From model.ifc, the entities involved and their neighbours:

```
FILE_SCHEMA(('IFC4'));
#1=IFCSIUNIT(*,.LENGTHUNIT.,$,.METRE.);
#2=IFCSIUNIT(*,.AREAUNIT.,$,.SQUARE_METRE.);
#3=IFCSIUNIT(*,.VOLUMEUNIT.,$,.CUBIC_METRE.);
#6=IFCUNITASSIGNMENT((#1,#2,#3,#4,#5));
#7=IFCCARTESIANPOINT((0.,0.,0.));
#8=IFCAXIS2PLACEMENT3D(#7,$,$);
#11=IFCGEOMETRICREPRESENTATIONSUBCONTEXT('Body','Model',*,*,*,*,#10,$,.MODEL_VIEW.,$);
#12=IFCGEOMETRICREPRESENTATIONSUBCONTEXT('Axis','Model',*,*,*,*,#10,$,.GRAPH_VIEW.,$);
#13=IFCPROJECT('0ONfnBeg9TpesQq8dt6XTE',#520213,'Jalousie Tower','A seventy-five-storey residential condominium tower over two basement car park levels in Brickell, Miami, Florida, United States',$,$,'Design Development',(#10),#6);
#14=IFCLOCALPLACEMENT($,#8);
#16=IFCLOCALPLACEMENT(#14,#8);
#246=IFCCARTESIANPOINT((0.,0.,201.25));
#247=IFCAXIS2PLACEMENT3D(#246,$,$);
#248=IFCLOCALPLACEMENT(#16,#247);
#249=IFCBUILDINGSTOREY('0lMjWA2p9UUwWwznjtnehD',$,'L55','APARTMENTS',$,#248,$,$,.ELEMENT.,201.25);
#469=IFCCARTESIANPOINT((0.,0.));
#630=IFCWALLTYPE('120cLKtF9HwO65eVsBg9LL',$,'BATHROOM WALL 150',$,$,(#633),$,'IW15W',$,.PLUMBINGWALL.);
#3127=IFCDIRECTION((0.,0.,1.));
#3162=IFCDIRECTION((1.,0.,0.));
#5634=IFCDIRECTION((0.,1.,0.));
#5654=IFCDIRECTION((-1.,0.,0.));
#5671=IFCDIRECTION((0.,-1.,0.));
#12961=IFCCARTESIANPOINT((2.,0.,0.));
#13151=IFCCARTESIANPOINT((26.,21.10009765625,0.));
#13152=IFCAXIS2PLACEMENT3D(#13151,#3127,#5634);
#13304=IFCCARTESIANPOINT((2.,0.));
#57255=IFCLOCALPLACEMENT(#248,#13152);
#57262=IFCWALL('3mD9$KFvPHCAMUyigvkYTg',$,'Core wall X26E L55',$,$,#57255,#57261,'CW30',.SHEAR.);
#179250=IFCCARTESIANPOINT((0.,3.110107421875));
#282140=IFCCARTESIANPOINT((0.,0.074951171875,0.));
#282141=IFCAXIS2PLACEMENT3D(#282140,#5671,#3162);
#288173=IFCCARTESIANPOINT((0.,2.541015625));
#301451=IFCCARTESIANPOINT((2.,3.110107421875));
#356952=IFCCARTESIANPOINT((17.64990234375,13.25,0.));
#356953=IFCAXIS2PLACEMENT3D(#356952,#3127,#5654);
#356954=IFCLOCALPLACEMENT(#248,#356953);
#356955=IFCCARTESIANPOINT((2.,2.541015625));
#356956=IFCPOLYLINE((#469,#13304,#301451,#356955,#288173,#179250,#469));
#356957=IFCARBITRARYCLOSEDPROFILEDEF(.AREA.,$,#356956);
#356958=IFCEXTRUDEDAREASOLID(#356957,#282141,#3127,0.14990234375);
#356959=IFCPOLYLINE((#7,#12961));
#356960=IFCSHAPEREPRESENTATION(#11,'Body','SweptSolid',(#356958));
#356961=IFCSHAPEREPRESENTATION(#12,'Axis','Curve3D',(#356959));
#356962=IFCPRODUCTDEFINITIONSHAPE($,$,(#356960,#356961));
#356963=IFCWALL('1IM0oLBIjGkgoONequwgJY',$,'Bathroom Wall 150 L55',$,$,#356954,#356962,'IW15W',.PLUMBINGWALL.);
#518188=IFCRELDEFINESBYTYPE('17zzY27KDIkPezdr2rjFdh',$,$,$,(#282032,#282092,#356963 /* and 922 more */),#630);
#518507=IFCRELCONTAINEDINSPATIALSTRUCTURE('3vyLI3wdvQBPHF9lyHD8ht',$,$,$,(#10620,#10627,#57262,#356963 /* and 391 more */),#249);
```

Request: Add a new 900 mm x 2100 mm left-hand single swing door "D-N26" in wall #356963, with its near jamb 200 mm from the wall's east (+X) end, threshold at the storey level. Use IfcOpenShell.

```python
import numpy as np
import ifcopenshell
import ifcopenshell.api.feature
import ifcopenshell.api.geometry
import ifcopenshell.api.root
import ifcopenshell.api.spatial
import ifcopenshell.geom
import ifcopenshell.util.element
import ifcopenshell.util.placement
import ifcopenshell.util.representation
import ifcopenshell.util.shape
import ifcopenshell.util.unit

model = ifcopenshell.open("model.ifc")
unit_scale = ifcopenshell.util.unit.calculate_unit_scale(model)
settings = ifcopenshell.geom.settings()


def volume(element):
    """Net volume in cubic metres, openings subtracted."""
    shape = ifcopenshell.geom.create_shape(settings, element)
    return ifcopenshell.util.shape.get_volume(shape.geometry)


wall = model.by_guid("1IM0oLBIjGkgoONequwgJY")
storey = ifcopenshell.util.element.get_container(wall, ifc_class="IfcBuildingStorey")
context = ifcopenshell.util.representation.get_context(model, "Model", "Body", "MODEL_VIEW")
before = volume(wall)

width, height, from_end, sill = 0.9, 2.1, 0.2, 0.0  # metres

# The wall runs along its own X axis, and the end named is its -X end.
wall_shape = ifcopenshell.geom.create_shape(settings, wall)
x, y, z = ifcopenshell.util.shape.get_vertices(wall_shape.geometry).T
start = x.min() + from_end
face, thickness = float(y.min()), float(y.max() - y.min())
wall_matrix = ifcopenshell.util.placement.get_local_placement(wall.ObjectPlacement)
level = ifcopenshell.util.placement.get_local_placement(storey.ObjectPlacement)[2, 3]


def in_wall(x, y):
    """Placement at x, y metres in the wall's axes, at sill height."""
    matrix = wall_matrix.copy()
    matrix[:, 3] = wall_matrix @ np.array([x / unit_scale, y / unit_scale, 0.0, 1.0])
    matrix[2, 3] = level + sill / unit_scale
    return matrix


# Opening: a box that overshoots both wall faces by 50 mm.
opening = ifcopenshell.api.root.create_entity(model, ifc_class="IfcOpeningElement", predefined_type="OPENING")
box = ifcopenshell.api.geometry.add_wall_representation(
    model, context=context, length=width, height=height, thickness=thickness + 0.1
)
ifcopenshell.api.geometry.assign_representation(model, product=opening, representation=box)
ifcopenshell.api.geometry.edit_object_placement(model, product=opening, matrix=in_wall(start, face - 0.05), is_si=False)
ifcopenshell.api.feature.add_feature(model, feature=opening, element=wall)

door = ifcopenshell.api.root.create_entity(model, ifc_class="IfcDoor", name="D-N26", predefined_type="DOOR")
door.OverallWidth, door.OverallHeight = width / unit_scale, height / unit_scale
door.OperationType = "SINGLE_SWING_LEFT"
body = ifcopenshell.api.geometry.add_door_representation(
    model,
    context=context,
    overall_width=door.OverallWidth,
    overall_height=door.OverallHeight,
    operation_type="SINGLE_SWING_LEFT",
    lining_properties={"LiningDepth": thickness / unit_scale, "ThresholdDepth": thickness / unit_scale},
)
ifcopenshell.api.geometry.assign_representation(model, product=door, representation=body)
ifcopenshell.api.spatial.assign_container(model, products=[door], relating_structure=storey)
ifcopenshell.api.feature.add_filling(model, opening=opening, element=door)

# The lining spans the wall, so the door starts at the wall face.
ifcopenshell.api.geometry.edit_object_placement(model, product=door, matrix=in_wall(start, face), is_si=False)

after = volume(wall)

print(f"wall volume {before:.3f} -> {after:.3f} m3")

model.write("model_rev.ifc")
```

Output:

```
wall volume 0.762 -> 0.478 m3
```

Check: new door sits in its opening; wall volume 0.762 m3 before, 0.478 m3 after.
